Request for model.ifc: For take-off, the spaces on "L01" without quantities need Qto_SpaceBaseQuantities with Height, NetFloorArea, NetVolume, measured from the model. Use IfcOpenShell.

First a look at what the model holds.

```python
import ifcopenshell
import ifcopenshell.util.element
import ifcopenshell.util.unit

model = ifcopenshell.open("model.ifc")
print(model.schema)
for unit_type in ("LENGTHUNIT", "AREAUNIT", "VOLUMEUNIT"):
    print(unit_type, ifcopenshell.util.unit.calculate_unit_scale(model, unit_type))
storey = next(s for s in model.by_type("IfcBuildingStorey") if s.Name == "L01")
spaces = [e for e in ifcopenshell.util.element.get_decomposition(storey) if e.is_a("IfcSpace")]
for e in sorted(spaces, key=lambda e: e.id()):
    print(e.id(), e.is_a(), e.Name, list(ifcopenshell.util.element.get_psets(e, qtos_only=True)), sep=" | ")
```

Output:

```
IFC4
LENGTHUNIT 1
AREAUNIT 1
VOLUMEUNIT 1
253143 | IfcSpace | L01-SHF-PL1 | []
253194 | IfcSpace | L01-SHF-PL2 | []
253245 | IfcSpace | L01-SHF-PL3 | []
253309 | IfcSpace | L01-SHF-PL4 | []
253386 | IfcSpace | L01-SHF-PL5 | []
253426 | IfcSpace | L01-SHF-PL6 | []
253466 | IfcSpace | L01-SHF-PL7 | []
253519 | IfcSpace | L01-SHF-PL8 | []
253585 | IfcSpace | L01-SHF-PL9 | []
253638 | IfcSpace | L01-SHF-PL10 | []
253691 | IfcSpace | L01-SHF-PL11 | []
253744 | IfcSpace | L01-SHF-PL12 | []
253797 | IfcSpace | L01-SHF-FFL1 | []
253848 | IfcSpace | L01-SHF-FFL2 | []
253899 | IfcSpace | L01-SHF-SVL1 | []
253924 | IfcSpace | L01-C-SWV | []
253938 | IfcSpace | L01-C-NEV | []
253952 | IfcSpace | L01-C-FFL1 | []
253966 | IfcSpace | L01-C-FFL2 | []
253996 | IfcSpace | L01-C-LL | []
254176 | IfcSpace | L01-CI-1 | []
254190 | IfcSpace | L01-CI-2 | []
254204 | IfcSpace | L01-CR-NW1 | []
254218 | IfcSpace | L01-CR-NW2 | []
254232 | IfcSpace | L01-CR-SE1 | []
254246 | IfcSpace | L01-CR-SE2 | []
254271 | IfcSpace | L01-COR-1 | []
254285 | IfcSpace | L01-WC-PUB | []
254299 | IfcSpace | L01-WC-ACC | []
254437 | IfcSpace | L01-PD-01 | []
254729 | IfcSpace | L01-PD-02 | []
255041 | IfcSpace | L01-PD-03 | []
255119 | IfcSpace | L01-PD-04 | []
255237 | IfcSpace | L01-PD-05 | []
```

```python
import ifcopenshell
import ifcopenshell.api.pset
import ifcopenshell.geom
import ifcopenshell.util.element
import ifcopenshell.util.shape
import ifcopenshell.util.unit

model = ifcopenshell.open("model.ifc")
unit_scale = ifcopenshell.util.unit.calculate_unit_scale(model)
area_scale = ifcopenshell.util.unit.calculate_unit_scale(model, "AREAUNIT")
volume_scale = ifcopenshell.util.unit.calculate_unit_scale(model, "VOLUMEUNIT")
settings = ifcopenshell.geom.settings()

storey = next(s for s in model.by_type("IfcBuildingStorey") if s.Name == "L01")
spaces = [e for e in ifcopenshell.util.element.get_decomposition(storey) if e.is_a("IfcSpace")]

for e in sorted(spaces, key=lambda e: e.id()):
    if ifcopenshell.util.element.get_psets(e, qtos_only=True, should_inherit=False):
        continue
    # Geometry comes back in metres, in the element's own axes.
    shape = ifcopenshell.geom.create_shape(settings, e)
    values = {
        "Height": ifcopenshell.util.shape.get_z(shape.geometry) / unit_scale,
        "NetFloorArea": ifcopenshell.util.shape.get_footprint_area(shape.geometry) / area_scale,
        "NetVolume": ifcopenshell.util.shape.get_volume(shape.geometry) / volume_scale,
    }
    qto = ifcopenshell.api.pset.add_qto(model, product=e, name="Qto_SpaceBaseQuantities")
    ifcopenshell.api.pset.edit_qto(model, qto=qto, properties=values)
    print(e.id(), {k: round(v, 3) for k, v in values.items()})

model.write("model_updated.ifc")
```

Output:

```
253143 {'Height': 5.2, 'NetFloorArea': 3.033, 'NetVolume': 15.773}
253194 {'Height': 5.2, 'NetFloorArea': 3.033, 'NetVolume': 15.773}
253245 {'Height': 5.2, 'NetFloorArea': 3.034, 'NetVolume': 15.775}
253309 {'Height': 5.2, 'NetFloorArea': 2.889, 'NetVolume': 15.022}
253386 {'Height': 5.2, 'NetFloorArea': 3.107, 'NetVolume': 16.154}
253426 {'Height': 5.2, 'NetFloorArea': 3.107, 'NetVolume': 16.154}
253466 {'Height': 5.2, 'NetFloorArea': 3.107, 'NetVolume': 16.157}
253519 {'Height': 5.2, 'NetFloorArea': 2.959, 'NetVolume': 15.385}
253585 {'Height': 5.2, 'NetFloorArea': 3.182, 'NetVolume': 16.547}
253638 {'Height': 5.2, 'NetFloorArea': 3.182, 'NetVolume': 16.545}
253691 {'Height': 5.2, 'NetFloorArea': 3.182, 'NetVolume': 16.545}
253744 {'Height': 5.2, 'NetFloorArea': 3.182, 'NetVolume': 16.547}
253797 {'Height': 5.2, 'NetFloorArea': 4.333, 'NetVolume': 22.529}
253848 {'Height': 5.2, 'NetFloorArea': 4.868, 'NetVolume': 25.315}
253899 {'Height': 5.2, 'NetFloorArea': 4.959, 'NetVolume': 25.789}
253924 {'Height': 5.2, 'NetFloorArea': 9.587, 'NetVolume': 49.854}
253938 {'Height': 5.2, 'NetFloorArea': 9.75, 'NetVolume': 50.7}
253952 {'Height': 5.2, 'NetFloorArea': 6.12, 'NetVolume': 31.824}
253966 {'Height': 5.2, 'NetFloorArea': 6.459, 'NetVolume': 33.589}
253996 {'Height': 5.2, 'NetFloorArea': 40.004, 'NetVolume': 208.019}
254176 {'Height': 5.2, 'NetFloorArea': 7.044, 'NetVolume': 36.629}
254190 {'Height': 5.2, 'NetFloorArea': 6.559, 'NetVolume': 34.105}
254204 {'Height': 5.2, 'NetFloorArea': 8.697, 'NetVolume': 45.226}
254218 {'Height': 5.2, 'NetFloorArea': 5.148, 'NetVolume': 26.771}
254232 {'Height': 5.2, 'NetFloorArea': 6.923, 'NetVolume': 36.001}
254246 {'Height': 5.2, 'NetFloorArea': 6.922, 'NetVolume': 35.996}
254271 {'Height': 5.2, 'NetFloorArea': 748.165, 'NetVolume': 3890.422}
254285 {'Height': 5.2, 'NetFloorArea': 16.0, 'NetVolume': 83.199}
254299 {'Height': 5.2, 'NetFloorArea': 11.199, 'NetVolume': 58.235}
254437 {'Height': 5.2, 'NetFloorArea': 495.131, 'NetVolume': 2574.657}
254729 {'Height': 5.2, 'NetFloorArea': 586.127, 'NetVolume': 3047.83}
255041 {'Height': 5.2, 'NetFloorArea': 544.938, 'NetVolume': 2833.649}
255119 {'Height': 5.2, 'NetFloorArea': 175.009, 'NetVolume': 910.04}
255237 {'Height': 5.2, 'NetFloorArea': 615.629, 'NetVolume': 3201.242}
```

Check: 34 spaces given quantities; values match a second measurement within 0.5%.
